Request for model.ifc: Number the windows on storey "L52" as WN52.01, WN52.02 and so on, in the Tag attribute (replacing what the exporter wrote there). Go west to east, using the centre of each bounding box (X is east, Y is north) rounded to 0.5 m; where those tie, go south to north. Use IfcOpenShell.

First a look at what the model holds.

```python
import ifcopenshell
import ifcopenshell.util.element
import ifcopenshell.util.placement

model = ifcopenshell.open("model.ifc")
print(model.schema)
storey = next(s for s in model.by_type("IfcBuildingStorey") if s.Name == "L52")
windows = [e for e in ifcopenshell.util.element.get_decomposition(storey) if e.is_a("IfcWindow")]
for e in sorted(windows, key=lambda e: e.id()):
    origin = ifcopenshell.util.placement.get_local_placement(e.ObjectPlacement)[:3, 3]
    print(e.id(), e.Tag, e.Name, origin.round(2) + 0.0, sep=" | ")
```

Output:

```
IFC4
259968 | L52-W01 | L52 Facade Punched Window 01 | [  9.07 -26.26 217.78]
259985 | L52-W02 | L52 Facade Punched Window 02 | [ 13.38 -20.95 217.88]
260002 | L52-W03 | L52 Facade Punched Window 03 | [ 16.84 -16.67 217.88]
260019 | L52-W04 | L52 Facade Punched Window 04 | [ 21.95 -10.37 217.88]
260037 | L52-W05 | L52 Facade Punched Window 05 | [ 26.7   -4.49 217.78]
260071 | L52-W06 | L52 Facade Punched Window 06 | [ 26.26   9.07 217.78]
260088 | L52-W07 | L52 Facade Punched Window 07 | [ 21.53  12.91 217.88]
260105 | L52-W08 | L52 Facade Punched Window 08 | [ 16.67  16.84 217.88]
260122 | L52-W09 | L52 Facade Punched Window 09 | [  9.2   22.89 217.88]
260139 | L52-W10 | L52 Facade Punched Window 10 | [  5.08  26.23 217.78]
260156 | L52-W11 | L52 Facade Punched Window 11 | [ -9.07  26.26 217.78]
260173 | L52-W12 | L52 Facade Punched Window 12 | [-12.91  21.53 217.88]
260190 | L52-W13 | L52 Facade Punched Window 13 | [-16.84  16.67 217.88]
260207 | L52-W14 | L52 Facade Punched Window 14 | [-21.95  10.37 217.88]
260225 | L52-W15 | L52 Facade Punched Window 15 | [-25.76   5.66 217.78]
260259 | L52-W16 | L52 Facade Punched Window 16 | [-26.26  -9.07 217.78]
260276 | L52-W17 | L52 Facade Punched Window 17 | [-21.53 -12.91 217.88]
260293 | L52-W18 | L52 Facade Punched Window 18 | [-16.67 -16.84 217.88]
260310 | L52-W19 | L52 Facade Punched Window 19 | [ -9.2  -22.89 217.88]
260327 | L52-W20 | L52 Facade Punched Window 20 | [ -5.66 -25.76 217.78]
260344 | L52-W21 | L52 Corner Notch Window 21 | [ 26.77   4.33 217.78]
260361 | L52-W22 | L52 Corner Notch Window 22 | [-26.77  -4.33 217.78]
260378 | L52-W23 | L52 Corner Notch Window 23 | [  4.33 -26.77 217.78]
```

```python
import ifcopenshell
import ifcopenshell.geom
import ifcopenshell.util.element
import ifcopenshell.util.shape

model = ifcopenshell.open("model.ifc")
settings = ifcopenshell.geom.settings()
settings.set("use-world-coords", True)


def centre(element):
    shape = ifcopenshell.geom.create_shape(settings, element)
    return ifcopenshell.util.shape.get_bbox_centroid(shape.geometry)


storey = next(s for s in model.by_type("IfcBuildingStorey") if s.Name == "L52")
windows = [e for e in ifcopenshell.util.element.get_decomposition(storey) if e.is_a("IfcWindow")]

# Insertion points can sit at a corner or the storey origin, so sort by the geometry (in metres).
centres = {e: centre(e) for e in windows}
windows.sort(key=lambda e: (round(centres[e][0] / 0.5), centres[e][1]))

for i, e in enumerate(windows, start=1):
    number = f"WN52.{i:02d}"
    e.Tag = number
    print(e.id(), number)

model.write("model_rev.ifc")
```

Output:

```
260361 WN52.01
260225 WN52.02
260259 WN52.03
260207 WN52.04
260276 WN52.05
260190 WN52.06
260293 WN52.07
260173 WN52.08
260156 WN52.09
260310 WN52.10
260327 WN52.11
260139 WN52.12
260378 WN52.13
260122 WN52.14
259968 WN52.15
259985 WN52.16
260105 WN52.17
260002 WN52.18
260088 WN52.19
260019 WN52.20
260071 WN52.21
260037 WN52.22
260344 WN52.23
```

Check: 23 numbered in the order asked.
